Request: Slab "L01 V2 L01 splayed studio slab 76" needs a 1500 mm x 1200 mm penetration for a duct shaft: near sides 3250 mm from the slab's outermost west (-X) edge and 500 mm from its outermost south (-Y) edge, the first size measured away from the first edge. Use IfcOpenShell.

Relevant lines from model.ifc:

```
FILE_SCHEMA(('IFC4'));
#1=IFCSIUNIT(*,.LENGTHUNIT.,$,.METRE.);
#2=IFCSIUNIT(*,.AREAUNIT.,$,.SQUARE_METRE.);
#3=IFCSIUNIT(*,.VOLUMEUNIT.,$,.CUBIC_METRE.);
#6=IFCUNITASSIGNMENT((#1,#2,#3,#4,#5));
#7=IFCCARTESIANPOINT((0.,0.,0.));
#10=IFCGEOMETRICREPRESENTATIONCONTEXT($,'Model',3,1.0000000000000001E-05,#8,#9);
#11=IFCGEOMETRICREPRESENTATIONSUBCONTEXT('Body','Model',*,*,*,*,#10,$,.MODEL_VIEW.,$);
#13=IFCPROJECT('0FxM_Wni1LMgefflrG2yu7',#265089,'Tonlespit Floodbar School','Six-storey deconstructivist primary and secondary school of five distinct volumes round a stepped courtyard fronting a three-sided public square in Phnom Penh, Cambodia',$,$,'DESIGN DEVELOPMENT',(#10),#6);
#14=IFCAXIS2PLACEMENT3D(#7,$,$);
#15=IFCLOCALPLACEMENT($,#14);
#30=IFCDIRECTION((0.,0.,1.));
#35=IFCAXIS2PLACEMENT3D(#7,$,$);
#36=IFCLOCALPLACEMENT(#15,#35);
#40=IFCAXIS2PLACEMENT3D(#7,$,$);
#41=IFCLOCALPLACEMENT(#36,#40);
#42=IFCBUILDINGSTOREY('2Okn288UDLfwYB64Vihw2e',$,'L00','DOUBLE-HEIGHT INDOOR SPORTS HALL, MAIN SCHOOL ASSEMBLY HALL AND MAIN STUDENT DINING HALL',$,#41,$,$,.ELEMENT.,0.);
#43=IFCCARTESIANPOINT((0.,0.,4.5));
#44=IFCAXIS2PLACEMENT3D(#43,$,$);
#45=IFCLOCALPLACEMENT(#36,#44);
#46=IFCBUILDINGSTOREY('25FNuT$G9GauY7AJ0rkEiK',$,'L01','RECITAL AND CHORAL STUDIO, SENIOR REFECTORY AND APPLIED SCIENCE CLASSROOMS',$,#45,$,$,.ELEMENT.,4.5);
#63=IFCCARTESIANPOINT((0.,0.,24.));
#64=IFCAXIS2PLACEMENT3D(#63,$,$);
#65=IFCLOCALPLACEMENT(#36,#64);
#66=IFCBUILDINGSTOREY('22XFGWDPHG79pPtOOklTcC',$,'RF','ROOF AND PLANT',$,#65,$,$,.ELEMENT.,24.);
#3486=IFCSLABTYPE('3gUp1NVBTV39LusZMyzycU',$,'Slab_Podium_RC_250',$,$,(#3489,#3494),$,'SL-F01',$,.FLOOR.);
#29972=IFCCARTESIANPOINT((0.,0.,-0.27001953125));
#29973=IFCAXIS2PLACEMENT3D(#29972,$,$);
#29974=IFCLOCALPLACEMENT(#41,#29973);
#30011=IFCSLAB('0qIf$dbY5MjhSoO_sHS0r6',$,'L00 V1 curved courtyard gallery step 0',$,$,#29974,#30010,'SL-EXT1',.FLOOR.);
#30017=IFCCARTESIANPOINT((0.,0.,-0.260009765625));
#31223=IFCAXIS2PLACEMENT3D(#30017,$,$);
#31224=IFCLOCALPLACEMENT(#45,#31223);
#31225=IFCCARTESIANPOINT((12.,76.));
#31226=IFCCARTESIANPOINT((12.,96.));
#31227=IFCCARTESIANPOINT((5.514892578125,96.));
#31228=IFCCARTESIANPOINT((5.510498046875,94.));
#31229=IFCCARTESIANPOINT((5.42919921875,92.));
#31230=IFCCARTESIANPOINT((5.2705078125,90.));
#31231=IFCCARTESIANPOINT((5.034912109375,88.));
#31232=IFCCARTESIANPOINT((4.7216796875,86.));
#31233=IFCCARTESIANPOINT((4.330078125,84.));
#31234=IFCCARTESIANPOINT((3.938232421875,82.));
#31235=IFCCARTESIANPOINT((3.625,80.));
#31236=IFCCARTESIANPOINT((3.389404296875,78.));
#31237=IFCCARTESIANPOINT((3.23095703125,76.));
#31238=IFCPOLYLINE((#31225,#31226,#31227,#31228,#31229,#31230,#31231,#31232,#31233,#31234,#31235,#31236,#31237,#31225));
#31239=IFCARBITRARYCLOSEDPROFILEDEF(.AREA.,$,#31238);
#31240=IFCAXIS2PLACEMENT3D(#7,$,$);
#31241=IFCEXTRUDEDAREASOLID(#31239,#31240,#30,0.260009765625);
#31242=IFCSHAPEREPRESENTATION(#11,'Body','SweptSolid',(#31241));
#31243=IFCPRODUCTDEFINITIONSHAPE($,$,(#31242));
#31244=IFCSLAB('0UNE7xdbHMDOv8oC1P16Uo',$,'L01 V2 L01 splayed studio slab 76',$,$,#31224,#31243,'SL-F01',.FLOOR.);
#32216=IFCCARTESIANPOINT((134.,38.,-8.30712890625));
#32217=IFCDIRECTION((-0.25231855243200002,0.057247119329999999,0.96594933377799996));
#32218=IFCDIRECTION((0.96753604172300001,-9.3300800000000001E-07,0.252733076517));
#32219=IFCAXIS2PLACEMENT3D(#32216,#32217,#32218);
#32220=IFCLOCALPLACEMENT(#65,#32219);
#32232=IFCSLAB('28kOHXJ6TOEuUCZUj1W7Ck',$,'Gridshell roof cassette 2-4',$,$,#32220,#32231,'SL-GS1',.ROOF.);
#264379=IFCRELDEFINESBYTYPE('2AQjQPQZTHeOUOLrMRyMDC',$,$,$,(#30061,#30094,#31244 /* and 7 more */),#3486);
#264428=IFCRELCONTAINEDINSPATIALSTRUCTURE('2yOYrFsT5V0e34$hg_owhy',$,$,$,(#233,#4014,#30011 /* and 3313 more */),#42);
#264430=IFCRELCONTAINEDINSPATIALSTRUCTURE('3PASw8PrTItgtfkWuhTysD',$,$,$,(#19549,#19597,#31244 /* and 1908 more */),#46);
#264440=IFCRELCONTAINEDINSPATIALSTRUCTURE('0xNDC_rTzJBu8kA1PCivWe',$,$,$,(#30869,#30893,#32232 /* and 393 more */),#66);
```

```python
import numpy as np
import ifcopenshell
import ifcopenshell.api.feature
import ifcopenshell.api.geometry
import ifcopenshell.api.root
import ifcopenshell.geom
import ifcopenshell.util.placement
import ifcopenshell.util.representation
import ifcopenshell.util.shape
import ifcopenshell.util.unit

model = ifcopenshell.open("model.ifc")
unit_scale = ifcopenshell.util.unit.calculate_unit_scale(model)
settings = ifcopenshell.geom.settings()


def volume(element):
    """Net volume in cubic metres, openings subtracted."""
    shape = ifcopenshell.geom.create_shape(settings, element)
    return ifcopenshell.util.shape.get_volume(shape.geometry)


slab = model.by_id(31244)
before = volume(slab)

# Extent in the slab's own axes, in metres. The edges named are its -X and -Y sides.
slab_shape = ifcopenshell.geom.create_shape(settings, slab)
vertices = ifcopenshell.util.shape.get_vertices(slab_shape.geometry)
x_min, y_min, bottom = vertices.min(axis=0)
top = vertices[:, 2].max()

opening = ifcopenshell.api.root.create_entity(model, ifc_class="IfcOpeningElement", name="Duct shaft opening", predefined_type="OPENING")
context = ifcopenshell.util.representation.get_context(model, "Model", "Body", "MODEL_VIEW")
width, depth = 1.5, 1.2
outline = [(0.0, 0.0), (width, 0.0), (width, depth), (0.0, depth), (0.0, 0.0)]
# Overshoot both faces by 50 mm so the cut is clean.
shape = ifcopenshell.api.geometry.add_slab_representation(
    model, context=context, depth=top - bottom + 0.1, polyline=outline
)
ifcopenshell.api.geometry.assign_representation(model, product=opening, representation=shape)

matrix = ifcopenshell.util.placement.get_local_placement(slab.ObjectPlacement)
matrix[:, 3] = matrix @ np.append(np.array([x_min + 3.25, y_min + 0.5, bottom - 0.05]) / unit_scale, 1.0)
ifcopenshell.api.geometry.edit_object_placement(model, product=opening, matrix=matrix, is_si=False)
ifcopenshell.api.feature.add_feature(model, feature=opening, element=slab)

after = volume(slab)

print(f"slab volume {before:.3f} -> {after:.3f} m3")

model.write("model-out.ifc")
```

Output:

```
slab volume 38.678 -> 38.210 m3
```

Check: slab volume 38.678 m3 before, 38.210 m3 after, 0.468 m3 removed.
